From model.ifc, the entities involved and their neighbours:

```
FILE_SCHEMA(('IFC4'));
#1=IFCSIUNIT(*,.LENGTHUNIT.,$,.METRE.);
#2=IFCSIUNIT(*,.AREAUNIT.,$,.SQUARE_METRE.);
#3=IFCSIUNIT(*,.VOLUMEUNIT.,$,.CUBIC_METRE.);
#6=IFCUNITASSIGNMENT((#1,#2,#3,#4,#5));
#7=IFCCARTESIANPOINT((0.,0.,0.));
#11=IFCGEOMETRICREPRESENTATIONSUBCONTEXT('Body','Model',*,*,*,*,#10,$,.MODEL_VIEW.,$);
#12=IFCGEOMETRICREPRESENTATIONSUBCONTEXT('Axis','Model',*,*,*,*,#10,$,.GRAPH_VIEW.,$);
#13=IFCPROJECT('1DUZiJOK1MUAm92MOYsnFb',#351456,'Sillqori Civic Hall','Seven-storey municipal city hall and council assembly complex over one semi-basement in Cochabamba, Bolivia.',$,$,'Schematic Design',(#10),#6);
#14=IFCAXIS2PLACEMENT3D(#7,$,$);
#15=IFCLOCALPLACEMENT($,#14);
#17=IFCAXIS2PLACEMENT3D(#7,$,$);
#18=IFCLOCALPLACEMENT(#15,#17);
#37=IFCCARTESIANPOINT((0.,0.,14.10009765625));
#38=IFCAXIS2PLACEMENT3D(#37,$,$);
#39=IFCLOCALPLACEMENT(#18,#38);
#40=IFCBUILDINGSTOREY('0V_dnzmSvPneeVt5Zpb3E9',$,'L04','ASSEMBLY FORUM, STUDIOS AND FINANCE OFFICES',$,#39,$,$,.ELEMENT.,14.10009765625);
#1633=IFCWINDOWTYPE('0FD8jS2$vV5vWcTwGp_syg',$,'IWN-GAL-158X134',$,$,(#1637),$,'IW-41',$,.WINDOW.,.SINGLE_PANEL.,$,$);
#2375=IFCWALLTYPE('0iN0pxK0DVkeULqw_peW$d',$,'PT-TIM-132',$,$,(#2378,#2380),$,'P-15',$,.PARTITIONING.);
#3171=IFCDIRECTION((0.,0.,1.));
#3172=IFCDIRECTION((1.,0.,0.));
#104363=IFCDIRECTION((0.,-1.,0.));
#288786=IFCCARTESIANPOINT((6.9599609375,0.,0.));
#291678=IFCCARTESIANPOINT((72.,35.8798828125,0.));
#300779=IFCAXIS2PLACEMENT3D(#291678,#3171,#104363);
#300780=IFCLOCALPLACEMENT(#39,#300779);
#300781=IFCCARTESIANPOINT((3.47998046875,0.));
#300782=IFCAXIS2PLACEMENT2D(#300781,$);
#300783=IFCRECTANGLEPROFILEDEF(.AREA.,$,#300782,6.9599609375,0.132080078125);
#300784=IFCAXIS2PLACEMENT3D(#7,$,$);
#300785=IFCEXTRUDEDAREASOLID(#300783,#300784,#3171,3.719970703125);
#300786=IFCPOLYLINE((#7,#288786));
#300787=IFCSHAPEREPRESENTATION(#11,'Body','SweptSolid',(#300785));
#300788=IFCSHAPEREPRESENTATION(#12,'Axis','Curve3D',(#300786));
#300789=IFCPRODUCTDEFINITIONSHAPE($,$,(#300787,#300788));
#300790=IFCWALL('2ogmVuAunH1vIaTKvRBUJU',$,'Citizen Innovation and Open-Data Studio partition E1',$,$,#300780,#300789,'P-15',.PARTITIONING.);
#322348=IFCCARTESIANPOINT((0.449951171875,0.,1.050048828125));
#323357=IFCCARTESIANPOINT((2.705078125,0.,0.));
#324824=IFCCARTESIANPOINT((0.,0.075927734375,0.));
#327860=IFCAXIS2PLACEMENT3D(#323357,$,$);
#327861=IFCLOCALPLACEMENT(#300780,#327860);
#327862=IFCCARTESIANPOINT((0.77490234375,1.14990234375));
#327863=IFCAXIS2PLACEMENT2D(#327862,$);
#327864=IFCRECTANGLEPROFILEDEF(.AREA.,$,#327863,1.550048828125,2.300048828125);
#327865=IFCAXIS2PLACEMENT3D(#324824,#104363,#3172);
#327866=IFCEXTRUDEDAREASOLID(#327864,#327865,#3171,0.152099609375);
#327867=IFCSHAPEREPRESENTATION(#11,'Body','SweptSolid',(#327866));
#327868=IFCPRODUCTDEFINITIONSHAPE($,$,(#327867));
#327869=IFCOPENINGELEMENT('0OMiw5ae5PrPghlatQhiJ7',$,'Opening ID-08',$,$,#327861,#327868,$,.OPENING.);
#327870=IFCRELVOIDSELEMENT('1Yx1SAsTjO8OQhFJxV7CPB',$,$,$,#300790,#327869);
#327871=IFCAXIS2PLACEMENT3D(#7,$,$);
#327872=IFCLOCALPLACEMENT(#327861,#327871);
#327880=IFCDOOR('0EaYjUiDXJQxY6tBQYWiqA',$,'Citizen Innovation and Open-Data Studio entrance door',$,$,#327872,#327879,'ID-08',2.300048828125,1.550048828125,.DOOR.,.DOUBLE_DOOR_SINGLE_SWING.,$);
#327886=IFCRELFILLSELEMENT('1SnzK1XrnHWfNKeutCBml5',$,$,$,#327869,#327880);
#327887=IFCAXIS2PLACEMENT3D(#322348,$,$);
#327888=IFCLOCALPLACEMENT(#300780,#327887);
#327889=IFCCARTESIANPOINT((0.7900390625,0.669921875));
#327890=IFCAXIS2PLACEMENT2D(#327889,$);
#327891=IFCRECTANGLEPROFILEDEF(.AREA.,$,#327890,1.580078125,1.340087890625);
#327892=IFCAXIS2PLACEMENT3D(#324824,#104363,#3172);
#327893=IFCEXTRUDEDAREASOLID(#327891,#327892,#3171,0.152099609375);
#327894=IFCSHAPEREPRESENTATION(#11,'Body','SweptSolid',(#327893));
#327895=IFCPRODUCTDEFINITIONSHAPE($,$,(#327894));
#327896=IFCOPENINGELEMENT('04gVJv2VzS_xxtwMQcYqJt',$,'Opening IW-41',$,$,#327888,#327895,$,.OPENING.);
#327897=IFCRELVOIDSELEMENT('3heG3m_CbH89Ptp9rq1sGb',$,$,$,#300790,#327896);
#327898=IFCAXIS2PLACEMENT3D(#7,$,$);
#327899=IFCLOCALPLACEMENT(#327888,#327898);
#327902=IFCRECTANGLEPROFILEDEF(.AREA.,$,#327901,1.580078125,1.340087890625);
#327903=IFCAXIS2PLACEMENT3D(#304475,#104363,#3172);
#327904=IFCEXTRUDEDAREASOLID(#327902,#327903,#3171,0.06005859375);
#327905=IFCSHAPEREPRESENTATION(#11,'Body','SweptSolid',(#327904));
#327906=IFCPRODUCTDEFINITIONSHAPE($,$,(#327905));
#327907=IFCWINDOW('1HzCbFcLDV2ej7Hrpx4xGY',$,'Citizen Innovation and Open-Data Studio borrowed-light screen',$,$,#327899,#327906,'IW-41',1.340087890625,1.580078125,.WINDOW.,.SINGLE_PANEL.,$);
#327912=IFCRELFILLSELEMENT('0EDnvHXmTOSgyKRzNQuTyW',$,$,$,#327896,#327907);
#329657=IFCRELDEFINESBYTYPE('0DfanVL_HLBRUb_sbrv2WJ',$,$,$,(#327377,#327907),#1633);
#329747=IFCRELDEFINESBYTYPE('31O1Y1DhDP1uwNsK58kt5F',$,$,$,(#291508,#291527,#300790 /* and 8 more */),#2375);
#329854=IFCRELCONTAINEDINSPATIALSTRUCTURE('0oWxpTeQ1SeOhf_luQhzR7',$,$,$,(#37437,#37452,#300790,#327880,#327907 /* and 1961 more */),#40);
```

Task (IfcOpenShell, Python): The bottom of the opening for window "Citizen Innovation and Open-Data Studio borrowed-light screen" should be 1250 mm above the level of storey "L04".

```python
import numpy as np
import ifcopenshell
import ifcopenshell.api.geometry
import ifcopenshell.geom
import ifcopenshell.util.element
import ifcopenshell.util.placement
import ifcopenshell.util.shape
import ifcopenshell.util.unit

model = ifcopenshell.open("model.ifc")
unit_scale = ifcopenshell.util.unit.calculate_unit_scale(model)

window = model.by_guid("1HzCbFcLDV2ej7Hrpx4xGY")
opening = window.FillsVoids[0].RelatingOpeningElement
storey = ifcopenshell.util.element.get_container(window, ifc_class="IfcBuildingStorey")
level = ifcopenshell.util.placement.get_local_placement(storey.ObjectPlacement)[2, 3]

# The opening's origin need not be at the sill, so measure its lowest point.
shape = ifcopenshell.geom.create_shape(ifcopenshell.geom.settings(), opening)
bottom = ifcopenshell.util.shape.get_shape_bottom_elevation(shape, shape.geometry) / unit_scale
dz = level + 1.25 - bottom

shift = np.array([0.0, 0.0, dz])
# The window is placed relative to its opening, so it follows when the opening moves.
matrix = ifcopenshell.util.placement.get_local_placement(opening.ObjectPlacement)
matrix[:3, 3] += shift
ifcopenshell.api.geometry.edit_object_placement(
    model, product=opening, matrix=matrix, is_si=False, should_transform_children=True
)

print(f"moved by {dz * unit_scale:+.3f} m")

model.write("model_rev.ifc")
```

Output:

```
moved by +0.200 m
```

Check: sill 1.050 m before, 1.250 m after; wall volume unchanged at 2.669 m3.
